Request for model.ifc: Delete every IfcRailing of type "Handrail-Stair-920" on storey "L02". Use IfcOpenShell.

First a look at what the model holds.

```python
import ifcopenshell
import ifcopenshell.util.element

model = ifcopenshell.open("model.ifc")
print(model.schema)
storey = next(s for s in model.by_type("IfcBuildingStorey") if s.Name == "L02")
railings = [e for e in ifcopenshell.util.element.get_decomposition(storey) if e.is_a("IfcRailing")]
seen = {}
for e in railings:
    element_type = ifcopenshell.util.element.get_type(e)
    name = element_type.Name if element_type not in (None, e) else None
    seen[name] = seen.get(name, 0) + 1
for name, count in sorted(seen.items(), key=str):
    print(count, "x", name)
```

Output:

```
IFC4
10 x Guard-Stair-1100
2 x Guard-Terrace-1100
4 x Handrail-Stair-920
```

```python
import ifcopenshell
import ifcopenshell.api.root
import ifcopenshell.util.element

model = ifcopenshell.open("model.ifc")

storey = next(s for s in model.by_type("IfcBuildingStorey") if s.Name == "L02")
railings = [e for e in ifcopenshell.util.element.get_decomposition(storey) if e.is_a("IfcRailing")]
targets = [e for e in railings if (t := ifcopenshell.util.element.get_type(e)) not in (None, e) and t.Name == "Handrail-Stair-920"]

for e in targets:
    ifcopenshell.api.root.remove_product(model, product=e)
print(len(targets), "removed")

model.write("model_updated.ifc")
```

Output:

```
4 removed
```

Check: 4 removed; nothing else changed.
